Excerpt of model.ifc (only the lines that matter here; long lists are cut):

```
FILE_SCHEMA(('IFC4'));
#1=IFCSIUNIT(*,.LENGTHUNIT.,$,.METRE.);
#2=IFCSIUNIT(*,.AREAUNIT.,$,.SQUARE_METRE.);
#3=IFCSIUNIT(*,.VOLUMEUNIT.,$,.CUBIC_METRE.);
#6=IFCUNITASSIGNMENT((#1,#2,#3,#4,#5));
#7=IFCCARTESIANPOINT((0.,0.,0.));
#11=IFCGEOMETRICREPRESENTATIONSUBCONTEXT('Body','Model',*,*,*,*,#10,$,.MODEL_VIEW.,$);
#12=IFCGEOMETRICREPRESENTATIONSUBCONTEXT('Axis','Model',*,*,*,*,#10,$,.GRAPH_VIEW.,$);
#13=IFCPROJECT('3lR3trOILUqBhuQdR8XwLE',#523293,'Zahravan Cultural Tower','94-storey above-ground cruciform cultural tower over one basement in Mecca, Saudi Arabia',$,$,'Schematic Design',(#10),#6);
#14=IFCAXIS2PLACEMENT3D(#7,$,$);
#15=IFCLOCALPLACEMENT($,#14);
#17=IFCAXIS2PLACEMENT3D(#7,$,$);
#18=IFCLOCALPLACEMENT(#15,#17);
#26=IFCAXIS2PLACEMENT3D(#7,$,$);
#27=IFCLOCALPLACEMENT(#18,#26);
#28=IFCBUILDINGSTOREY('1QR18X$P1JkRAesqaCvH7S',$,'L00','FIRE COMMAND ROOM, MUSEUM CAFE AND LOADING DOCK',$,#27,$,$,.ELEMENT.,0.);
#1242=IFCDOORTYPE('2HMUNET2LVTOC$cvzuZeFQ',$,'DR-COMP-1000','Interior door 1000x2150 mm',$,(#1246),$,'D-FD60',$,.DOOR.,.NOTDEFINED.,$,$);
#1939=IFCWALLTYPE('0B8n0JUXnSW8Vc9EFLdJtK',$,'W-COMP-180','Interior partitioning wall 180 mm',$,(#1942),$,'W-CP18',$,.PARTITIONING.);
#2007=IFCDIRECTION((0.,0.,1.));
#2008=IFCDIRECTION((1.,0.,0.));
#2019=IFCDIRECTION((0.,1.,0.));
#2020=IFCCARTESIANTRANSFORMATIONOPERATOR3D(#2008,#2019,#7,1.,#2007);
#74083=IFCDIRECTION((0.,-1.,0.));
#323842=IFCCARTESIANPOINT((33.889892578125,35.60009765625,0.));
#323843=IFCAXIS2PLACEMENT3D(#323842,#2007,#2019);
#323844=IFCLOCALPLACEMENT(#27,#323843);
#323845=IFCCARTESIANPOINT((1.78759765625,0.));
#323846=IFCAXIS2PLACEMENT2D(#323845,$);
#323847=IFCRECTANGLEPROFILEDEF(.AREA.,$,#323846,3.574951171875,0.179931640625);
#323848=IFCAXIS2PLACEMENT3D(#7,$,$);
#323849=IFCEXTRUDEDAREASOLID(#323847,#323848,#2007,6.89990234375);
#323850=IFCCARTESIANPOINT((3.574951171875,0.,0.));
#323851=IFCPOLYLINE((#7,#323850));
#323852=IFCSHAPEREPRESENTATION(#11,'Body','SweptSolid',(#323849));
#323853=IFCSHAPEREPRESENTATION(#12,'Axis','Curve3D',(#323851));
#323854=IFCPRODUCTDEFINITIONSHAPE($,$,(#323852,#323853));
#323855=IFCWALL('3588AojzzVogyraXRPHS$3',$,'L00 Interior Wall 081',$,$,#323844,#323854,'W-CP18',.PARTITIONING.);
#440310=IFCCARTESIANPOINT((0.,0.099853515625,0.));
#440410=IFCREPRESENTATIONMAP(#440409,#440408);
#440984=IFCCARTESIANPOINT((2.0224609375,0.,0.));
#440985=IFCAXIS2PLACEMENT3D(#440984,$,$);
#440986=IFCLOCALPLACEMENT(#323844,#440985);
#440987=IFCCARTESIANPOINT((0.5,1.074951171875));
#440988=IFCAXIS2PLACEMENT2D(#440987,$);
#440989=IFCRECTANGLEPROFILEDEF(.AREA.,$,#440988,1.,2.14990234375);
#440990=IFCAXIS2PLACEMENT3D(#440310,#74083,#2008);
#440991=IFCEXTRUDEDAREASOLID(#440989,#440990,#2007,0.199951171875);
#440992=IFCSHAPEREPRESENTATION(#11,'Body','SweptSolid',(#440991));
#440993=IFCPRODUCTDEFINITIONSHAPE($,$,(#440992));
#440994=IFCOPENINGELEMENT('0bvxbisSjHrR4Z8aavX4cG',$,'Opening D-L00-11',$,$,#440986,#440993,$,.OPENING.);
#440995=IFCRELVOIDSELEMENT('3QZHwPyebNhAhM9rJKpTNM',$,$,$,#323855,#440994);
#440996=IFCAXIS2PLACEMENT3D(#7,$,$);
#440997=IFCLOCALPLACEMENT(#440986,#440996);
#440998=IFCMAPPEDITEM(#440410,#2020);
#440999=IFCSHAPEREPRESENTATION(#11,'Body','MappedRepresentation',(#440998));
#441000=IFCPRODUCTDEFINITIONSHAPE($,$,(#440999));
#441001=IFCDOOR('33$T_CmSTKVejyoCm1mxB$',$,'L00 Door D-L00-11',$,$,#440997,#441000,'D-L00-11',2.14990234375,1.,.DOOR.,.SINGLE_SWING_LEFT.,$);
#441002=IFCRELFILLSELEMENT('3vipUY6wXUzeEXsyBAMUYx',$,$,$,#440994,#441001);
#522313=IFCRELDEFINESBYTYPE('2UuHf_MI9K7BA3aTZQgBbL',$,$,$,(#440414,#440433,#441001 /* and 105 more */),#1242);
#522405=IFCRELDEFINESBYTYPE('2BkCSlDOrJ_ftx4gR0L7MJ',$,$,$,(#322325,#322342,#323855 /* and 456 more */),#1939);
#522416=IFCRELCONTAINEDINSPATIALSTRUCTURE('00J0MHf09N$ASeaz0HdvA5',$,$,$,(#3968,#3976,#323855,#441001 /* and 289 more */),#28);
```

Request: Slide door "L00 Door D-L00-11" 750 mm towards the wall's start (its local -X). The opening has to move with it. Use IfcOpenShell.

```python
import ifcopenshell
import ifcopenshell.api.geometry
import ifcopenshell.util.placement
import ifcopenshell.util.unit

model = ifcopenshell.open("model.ifc")
unit_scale = ifcopenshell.util.unit.calculate_unit_scale(model)

door = model.by_id(441001)
opening = door.FillsVoids[0].RelatingOpeningElement
wall = opening.VoidsElements[0].RelatingBuildingElement

wall_matrix = ifcopenshell.util.placement.get_local_placement(wall.ObjectPlacement)
shift = wall_matrix[:3, 0] * -0.75 / unit_scale
before = ifcopenshell.util.placement.get_local_placement(door.ObjectPlacement)[:3, 3].copy()

# The door is placed relative to its opening, so it follows when the opening moves.
matrix = ifcopenshell.util.placement.get_local_placement(opening.ObjectPlacement)
matrix[:3, 3] += shift
ifcopenshell.api.geometry.edit_object_placement(
    model, product=opening, matrix=matrix, is_si=False, should_transform_children=True
)

after = ifcopenshell.util.placement.get_local_placement(door.ObjectPlacement)[:3, 3]
print("door moved by", (after - before).round(3) + 0.0)

model.write("model_v2.ifc")
```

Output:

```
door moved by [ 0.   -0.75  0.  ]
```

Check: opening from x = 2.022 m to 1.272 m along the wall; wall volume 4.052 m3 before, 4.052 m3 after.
